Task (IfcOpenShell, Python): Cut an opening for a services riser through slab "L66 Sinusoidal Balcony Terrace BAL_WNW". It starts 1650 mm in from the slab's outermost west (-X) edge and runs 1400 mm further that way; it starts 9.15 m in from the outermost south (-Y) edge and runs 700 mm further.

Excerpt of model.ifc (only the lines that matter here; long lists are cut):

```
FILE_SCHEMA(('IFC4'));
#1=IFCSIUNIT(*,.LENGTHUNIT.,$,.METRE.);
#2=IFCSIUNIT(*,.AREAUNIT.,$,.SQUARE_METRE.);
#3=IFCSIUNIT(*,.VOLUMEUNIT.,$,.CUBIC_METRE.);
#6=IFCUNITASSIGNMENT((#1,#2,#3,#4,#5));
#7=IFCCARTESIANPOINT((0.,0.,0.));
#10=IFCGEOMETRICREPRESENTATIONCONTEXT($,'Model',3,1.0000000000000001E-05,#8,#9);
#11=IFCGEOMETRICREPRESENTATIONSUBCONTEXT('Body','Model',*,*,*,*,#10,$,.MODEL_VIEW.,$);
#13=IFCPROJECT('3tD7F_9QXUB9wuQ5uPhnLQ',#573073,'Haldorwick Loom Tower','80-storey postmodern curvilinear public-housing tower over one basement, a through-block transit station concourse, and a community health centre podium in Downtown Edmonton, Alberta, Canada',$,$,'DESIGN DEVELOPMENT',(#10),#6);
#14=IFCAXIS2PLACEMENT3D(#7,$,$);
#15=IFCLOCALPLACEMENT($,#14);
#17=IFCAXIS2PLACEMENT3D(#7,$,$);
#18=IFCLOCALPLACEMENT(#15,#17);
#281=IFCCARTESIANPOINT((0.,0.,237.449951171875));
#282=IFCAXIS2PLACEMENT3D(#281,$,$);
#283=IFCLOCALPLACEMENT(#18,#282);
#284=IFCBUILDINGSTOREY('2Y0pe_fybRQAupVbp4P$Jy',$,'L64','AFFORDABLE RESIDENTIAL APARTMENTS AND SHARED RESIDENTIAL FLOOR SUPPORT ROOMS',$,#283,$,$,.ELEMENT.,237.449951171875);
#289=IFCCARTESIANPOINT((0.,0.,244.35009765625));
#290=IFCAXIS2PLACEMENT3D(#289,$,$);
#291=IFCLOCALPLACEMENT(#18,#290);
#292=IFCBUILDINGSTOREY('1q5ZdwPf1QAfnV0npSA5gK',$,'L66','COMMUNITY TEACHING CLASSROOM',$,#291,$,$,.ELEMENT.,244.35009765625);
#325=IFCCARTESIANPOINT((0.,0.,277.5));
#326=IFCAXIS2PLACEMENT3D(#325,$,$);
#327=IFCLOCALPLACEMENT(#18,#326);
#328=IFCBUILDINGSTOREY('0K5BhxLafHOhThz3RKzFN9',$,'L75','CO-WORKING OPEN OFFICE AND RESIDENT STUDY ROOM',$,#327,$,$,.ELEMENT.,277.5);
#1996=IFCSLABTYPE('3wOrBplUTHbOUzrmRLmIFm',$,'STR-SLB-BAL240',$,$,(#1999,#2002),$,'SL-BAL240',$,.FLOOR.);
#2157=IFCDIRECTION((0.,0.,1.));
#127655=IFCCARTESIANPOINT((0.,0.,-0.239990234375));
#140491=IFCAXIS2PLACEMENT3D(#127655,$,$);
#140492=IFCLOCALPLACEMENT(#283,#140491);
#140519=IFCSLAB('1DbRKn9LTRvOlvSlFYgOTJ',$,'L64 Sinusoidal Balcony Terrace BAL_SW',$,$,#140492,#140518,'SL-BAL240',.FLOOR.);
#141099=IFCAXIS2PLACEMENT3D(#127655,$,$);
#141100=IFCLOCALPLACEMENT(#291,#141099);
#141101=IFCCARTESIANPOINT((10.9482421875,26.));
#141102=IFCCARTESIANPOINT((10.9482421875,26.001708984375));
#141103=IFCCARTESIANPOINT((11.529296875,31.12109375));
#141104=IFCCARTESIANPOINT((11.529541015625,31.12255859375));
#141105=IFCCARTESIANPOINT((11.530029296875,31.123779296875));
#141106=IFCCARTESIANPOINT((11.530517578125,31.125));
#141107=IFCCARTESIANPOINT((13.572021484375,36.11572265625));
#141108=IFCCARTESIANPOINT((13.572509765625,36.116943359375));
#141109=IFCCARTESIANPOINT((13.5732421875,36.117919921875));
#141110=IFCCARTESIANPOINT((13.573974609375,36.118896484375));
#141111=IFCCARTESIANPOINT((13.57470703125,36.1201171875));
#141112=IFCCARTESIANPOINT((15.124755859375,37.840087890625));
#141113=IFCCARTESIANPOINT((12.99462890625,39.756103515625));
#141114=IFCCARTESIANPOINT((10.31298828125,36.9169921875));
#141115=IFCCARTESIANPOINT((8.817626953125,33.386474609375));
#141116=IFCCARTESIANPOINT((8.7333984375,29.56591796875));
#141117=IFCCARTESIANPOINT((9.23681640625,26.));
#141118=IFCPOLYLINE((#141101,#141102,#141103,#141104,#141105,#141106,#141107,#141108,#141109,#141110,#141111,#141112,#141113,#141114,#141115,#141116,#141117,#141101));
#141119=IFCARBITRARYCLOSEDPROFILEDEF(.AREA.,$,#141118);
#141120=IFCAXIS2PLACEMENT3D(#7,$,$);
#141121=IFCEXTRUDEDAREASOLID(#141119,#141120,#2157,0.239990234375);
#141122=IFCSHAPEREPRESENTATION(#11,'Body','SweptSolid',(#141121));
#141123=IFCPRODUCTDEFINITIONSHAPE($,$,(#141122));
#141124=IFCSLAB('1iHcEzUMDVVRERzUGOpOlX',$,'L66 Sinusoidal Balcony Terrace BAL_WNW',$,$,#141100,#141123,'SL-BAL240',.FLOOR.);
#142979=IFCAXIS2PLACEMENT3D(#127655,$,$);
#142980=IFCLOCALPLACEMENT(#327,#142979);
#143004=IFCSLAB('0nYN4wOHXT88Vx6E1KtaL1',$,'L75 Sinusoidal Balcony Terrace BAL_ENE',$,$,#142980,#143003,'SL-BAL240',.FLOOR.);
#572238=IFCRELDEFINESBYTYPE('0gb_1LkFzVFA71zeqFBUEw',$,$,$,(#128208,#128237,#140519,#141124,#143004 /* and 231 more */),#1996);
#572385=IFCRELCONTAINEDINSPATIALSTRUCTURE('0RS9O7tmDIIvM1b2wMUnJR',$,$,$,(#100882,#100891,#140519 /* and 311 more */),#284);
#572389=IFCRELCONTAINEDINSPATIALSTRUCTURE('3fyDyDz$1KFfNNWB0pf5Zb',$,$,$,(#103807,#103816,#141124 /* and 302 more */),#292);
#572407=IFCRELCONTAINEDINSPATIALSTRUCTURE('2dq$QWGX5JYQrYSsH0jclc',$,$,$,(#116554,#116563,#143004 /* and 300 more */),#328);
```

```python
import numpy as np
import ifcopenshell
import ifcopenshell.api.feature
import ifcopenshell.api.geometry
import ifcopenshell.api.root
import ifcopenshell.geom
import ifcopenshell.util.placement
import ifcopenshell.util.representation
import ifcopenshell.util.shape
import ifcopenshell.util.unit

model = ifcopenshell.open("model.ifc")
unit_scale = ifcopenshell.util.unit.calculate_unit_scale(model)
settings = ifcopenshell.geom.settings()


def volume(element):
    """Net volume in cubic metres, openings subtracted."""
    shape = ifcopenshell.geom.create_shape(settings, element)
    return ifcopenshell.util.shape.get_volume(shape.geometry)


slab = model.by_id(141124)
before = volume(slab)

# Extent in the slab's own axes, in metres. The edges named are its -X and -Y sides.
slab_shape = ifcopenshell.geom.create_shape(settings, slab)
vertices = ifcopenshell.util.shape.get_vertices(slab_shape.geometry)
x_min, y_min, bottom = vertices.min(axis=0)
top = vertices[:, 2].max()

opening = ifcopenshell.api.root.create_entity(model, ifc_class="IfcOpeningElement", name="Services riser opening", predefined_type="OPENING")
context = ifcopenshell.util.representation.get_context(model, "Model", "Body", "MODEL_VIEW")
width, depth = 1.4, 0.7
outline = [(0.0, 0.0), (width, 0.0), (width, depth), (0.0, depth), (0.0, 0.0)]
# Overshoot both faces by 50 mm so the cut is clean.
shape = ifcopenshell.api.geometry.add_slab_representation(
    model, context=context, depth=top - bottom + 0.1, polyline=outline
)
ifcopenshell.api.geometry.assign_representation(model, product=opening, representation=shape)

matrix = ifcopenshell.util.placement.get_local_placement(slab.ObjectPlacement)
matrix[:, 3] = matrix @ np.append(np.array([x_min + 1.65, y_min + 9.15, bottom - 0.05]) / unit_scale, 1.0)
ifcopenshell.api.geometry.edit_object_placement(model, product=opening, matrix=matrix, is_si=False)
ifcopenshell.api.feature.add_feature(model, feature=opening, element=slab)

after = volume(slab)

print(f"slab volume {before:.3f} -> {after:.3f} m3")

model.write("model_v2.ifc")
```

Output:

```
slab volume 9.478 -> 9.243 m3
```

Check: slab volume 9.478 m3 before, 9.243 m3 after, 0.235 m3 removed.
